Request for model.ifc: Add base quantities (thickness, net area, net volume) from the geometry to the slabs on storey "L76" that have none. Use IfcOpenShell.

First a look at what the model holds.

```python
import ifcopenshell
import ifcopenshell.util.element
import ifcopenshell.util.unit

model = ifcopenshell.open("model.ifc")
print(model.schema)
for unit_type in ("LENGTHUNIT", "AREAUNIT", "VOLUMEUNIT"):
    print(unit_type, ifcopenshell.util.unit.calculate_unit_scale(model, unit_type))
storey = next(s for s in model.by_type("IfcBuildingStorey") if s.Name == "L76")
slabs = [e for e in ifcopenshell.util.element.get_decomposition(storey) if e.is_a("IfcSlab")]
for e in sorted(slabs, key=lambda e: e.id()):
    print(e.id(), e.is_a(), e.Name, list(ifcopenshell.util.element.get_psets(e, qtos_only=True)), sep=" | ")
```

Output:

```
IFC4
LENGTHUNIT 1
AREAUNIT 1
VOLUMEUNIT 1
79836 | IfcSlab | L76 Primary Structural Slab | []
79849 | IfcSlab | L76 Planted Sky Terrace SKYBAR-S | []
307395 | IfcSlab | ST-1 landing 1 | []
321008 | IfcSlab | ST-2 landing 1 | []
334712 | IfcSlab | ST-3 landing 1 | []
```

```python
import ifcopenshell
import ifcopenshell.api.pset
import ifcopenshell.geom
import ifcopenshell.util.element
import ifcopenshell.util.shape
import ifcopenshell.util.unit

model = ifcopenshell.open("model.ifc")
unit_scale = ifcopenshell.util.unit.calculate_unit_scale(model)
area_scale = ifcopenshell.util.unit.calculate_unit_scale(model, "AREAUNIT")
volume_scale = ifcopenshell.util.unit.calculate_unit_scale(model, "VOLUMEUNIT")
settings = ifcopenshell.geom.settings()

storey = next(s for s in model.by_type("IfcBuildingStorey") if s.Name == "L76")
slabs = [e for e in ifcopenshell.util.element.get_decomposition(storey) if e.is_a("IfcSlab")]

for e in sorted(slabs, key=lambda e: e.id()):
    if ifcopenshell.util.element.get_psets(e, qtos_only=True, should_inherit=False):
        continue
    # Geometry comes back in metres, in the element's own axes.
    shape = ifcopenshell.geom.create_shape(settings, e)
    values = {
        "Width": ifcopenshell.util.shape.get_z(shape.geometry) / unit_scale,
        "NetArea": ifcopenshell.util.shape.get_footprint_area(shape.geometry) / area_scale,
        "NetVolume": ifcopenshell.util.shape.get_volume(shape.geometry) / volume_scale,
    }
    qto = ifcopenshell.api.pset.add_qto(model, product=e, name="Qto_SlabBaseQuantities")
    ifcopenshell.api.pset.edit_qto(model, qto=qto, properties=values)
    print(e.id(), {k: round(v, 3) for k, v in values.items()})

model.write("model-out.ifc")
```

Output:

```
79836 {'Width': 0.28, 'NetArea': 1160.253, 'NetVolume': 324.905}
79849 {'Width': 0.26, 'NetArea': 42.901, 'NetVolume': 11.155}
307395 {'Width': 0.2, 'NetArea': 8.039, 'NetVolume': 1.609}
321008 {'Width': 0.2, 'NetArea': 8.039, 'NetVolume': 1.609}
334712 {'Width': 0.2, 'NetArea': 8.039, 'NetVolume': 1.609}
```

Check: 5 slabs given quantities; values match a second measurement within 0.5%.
